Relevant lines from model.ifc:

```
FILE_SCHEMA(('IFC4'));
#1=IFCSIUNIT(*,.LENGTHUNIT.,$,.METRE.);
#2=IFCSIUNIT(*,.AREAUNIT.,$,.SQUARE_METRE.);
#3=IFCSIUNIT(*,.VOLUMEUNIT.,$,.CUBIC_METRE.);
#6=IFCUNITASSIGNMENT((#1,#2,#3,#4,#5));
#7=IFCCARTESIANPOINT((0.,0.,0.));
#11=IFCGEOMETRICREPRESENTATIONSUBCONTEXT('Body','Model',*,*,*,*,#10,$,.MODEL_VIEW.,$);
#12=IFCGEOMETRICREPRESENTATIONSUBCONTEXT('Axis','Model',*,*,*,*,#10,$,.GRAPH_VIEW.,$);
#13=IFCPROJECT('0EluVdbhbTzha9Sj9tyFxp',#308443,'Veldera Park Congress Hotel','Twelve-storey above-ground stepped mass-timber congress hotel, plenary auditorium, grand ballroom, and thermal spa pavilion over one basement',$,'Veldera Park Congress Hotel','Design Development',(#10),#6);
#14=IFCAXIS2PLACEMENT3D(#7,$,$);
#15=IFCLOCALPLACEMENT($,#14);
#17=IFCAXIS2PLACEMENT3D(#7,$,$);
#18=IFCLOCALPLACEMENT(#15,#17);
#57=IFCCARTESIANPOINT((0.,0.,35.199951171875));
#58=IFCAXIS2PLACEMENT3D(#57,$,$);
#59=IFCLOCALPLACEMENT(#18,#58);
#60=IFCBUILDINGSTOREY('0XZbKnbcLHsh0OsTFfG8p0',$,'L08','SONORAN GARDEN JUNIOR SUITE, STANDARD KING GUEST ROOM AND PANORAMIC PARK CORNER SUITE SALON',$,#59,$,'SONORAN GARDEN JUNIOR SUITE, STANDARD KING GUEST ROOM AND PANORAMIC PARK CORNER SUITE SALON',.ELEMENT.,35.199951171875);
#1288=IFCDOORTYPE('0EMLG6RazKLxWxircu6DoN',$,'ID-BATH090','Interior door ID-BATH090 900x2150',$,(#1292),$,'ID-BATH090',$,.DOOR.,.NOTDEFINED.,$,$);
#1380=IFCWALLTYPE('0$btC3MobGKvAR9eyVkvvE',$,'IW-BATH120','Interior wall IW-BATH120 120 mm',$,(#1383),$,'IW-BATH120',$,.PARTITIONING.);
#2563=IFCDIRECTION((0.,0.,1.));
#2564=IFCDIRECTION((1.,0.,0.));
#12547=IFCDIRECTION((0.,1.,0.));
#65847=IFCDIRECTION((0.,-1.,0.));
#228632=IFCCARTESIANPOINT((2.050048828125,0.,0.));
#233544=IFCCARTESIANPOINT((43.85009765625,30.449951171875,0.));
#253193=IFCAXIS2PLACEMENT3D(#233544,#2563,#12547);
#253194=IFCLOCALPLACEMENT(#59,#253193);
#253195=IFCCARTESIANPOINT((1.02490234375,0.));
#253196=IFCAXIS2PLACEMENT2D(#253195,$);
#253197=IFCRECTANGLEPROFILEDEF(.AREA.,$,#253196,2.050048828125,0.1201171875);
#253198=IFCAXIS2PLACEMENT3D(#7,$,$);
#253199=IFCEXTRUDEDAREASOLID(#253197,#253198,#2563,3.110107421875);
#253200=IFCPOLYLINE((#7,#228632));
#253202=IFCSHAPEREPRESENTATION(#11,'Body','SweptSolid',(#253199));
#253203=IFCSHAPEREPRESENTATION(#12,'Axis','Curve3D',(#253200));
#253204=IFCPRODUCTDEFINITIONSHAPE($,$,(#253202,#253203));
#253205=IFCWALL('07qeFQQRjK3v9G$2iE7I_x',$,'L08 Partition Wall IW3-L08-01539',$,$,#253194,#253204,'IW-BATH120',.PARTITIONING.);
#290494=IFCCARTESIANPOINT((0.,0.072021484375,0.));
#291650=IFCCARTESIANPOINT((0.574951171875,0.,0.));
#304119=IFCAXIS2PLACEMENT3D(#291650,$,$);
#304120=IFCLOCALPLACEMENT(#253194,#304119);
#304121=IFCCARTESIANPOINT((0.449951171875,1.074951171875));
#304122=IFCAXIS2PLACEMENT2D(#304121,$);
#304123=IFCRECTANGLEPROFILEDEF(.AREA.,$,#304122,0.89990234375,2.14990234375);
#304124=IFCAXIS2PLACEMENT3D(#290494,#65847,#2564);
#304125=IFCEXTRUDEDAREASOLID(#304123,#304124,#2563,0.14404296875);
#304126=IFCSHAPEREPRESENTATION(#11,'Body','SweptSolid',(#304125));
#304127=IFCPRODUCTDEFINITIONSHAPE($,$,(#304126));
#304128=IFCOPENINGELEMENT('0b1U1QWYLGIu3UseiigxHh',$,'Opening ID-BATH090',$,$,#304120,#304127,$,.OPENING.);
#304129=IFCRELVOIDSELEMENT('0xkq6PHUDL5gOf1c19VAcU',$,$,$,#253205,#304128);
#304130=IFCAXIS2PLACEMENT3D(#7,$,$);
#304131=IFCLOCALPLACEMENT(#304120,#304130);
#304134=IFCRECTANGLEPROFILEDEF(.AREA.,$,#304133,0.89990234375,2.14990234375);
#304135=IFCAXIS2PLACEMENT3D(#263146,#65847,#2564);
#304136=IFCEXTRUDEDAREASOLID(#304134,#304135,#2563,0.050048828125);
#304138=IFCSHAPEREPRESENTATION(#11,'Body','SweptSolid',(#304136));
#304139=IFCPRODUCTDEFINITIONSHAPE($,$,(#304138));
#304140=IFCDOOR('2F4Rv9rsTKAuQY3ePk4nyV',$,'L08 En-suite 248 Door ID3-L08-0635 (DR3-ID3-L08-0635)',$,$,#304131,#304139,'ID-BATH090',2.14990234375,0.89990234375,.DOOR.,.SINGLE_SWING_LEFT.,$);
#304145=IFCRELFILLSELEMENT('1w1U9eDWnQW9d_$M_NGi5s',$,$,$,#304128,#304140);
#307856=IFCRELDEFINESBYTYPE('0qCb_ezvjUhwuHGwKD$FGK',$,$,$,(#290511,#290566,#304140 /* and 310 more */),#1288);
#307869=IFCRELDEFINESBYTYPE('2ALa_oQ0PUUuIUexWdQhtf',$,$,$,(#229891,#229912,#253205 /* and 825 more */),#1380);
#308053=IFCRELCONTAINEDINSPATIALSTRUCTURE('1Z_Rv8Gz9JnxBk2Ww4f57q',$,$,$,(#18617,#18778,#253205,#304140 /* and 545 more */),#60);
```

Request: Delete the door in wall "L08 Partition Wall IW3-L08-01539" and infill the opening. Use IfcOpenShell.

```python
import ifcopenshell
import ifcopenshell.api.feature
import ifcopenshell.api.root
import ifcopenshell.geom
import ifcopenshell.util.shape

model = ifcopenshell.open("model.ifc")
settings = ifcopenshell.geom.settings()


def volume(element):
    """Net volume in cubic metres, openings subtracted."""
    shape = ifcopenshell.geom.create_shape(settings, element)
    return ifcopenshell.util.shape.get_volume(shape.geometry)


door = model.by_guid("2F4Rv9rsTKAuQY3ePk4nyV")
opening = door.FillsVoids[0].RelatingOpeningElement
wall = opening.VoidsElements[0].RelatingBuildingElement
before = volume(wall)

ifcopenshell.api.root.remove_product(model, product=door)
ifcopenshell.api.feature.remove_feature(model, feature=opening)

after = volume(wall)

print(f"wall volume {before:.3f} -> {after:.3f} m3")

model.write("model_edited.ifc")
```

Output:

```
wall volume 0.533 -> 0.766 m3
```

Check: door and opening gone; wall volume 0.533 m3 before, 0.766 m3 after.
